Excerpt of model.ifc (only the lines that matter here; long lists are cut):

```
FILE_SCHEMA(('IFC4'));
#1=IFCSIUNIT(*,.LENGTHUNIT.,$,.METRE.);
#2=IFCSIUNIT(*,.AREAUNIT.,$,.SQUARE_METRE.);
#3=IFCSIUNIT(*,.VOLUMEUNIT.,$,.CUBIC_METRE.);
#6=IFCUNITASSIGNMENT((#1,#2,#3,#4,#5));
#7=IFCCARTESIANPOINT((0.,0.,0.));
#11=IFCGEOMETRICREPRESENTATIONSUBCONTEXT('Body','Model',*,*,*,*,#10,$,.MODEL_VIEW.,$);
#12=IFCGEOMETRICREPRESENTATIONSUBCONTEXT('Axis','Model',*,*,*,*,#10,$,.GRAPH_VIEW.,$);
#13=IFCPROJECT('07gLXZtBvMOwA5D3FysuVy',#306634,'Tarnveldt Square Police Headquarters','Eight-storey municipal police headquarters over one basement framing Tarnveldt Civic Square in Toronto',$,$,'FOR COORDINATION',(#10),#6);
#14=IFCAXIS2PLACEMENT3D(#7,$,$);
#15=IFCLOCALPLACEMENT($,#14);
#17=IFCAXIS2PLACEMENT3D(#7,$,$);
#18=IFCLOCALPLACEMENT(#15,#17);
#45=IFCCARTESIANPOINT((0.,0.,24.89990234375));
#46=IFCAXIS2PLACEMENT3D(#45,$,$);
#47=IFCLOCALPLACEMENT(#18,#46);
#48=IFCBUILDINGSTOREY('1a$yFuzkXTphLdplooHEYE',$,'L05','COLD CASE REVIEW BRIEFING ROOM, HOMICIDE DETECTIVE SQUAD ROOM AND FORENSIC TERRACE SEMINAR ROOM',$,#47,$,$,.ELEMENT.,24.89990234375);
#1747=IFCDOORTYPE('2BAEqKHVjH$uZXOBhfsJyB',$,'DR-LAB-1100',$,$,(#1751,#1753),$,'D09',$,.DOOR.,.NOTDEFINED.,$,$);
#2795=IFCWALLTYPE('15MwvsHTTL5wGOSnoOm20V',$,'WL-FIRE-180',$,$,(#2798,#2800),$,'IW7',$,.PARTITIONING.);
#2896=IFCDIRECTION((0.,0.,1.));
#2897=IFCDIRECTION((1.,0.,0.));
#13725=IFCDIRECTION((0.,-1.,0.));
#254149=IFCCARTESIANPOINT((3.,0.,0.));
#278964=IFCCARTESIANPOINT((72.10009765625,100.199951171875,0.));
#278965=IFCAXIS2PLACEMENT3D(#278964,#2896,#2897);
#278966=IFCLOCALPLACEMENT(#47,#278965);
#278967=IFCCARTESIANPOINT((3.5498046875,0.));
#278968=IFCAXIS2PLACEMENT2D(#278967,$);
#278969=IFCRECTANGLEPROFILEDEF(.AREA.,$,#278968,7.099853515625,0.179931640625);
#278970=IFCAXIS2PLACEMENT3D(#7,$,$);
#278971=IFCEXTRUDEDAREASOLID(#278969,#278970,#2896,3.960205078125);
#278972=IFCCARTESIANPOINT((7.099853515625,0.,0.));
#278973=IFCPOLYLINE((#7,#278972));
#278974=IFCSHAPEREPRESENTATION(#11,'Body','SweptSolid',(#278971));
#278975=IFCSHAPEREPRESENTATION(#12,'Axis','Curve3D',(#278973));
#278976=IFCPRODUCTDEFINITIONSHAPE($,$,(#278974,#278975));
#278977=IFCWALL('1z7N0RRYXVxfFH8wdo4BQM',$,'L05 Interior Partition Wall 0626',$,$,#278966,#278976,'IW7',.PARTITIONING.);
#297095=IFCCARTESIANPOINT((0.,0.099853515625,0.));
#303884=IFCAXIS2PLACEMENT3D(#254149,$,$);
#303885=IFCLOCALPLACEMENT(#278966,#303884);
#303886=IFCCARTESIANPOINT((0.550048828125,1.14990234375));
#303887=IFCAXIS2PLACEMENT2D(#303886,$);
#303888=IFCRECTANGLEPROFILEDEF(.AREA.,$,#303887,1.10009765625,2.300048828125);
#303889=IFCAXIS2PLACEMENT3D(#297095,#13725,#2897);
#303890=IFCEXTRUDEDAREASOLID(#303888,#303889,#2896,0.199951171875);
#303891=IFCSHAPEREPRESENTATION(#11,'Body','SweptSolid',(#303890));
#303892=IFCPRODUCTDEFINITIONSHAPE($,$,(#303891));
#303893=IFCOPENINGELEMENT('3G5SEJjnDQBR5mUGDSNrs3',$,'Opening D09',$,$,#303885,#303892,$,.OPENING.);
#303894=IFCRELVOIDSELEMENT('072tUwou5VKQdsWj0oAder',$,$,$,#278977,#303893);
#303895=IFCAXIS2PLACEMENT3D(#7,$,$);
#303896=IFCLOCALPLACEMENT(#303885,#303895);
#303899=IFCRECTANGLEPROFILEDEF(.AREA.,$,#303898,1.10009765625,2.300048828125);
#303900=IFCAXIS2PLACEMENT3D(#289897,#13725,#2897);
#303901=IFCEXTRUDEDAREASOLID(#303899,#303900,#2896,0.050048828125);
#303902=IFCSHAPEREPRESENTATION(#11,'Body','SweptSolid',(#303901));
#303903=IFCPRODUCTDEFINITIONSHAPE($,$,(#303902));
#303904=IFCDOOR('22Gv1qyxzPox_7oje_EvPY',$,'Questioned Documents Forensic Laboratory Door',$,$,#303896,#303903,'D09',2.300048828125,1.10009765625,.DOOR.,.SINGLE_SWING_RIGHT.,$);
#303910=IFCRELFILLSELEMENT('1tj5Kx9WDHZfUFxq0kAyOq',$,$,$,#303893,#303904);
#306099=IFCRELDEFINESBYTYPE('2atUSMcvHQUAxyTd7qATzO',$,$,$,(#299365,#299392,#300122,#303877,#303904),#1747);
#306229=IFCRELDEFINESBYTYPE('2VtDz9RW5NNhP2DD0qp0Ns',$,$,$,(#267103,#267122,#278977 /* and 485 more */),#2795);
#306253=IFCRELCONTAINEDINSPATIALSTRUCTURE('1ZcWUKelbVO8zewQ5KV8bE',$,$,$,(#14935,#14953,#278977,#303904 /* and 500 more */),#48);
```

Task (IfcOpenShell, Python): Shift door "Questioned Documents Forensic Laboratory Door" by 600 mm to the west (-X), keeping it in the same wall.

```python
import ifcopenshell
import ifcopenshell.api.geometry
import ifcopenshell.util.placement

model = ifcopenshell.open("model.ifc")

door = model.by_guid("22Gv1qyxzPox_7oje_EvPY")
opening = door.FillsVoids[0].RelatingOpeningElement
wall = opening.VoidsElements[0].RelatingBuildingElement

wall_matrix = ifcopenshell.util.placement.get_local_placement(wall.ObjectPlacement)
shift = wall_matrix[:3, 0] * -0.6
before = ifcopenshell.util.placement.get_local_placement(door.ObjectPlacement)[:3, 3].copy()

# The door is placed relative to its opening, so it follows when the opening moves.
matrix = ifcopenshell.util.placement.get_local_placement(opening.ObjectPlacement)
matrix[:3, 3] += shift
ifcopenshell.api.geometry.edit_object_placement(
    model, product=opening, matrix=matrix, is_si=False, should_transform_children=True
)

after = ifcopenshell.util.placement.get_local_placement(door.ObjectPlacement)[:3, 3]
print("door moved by", (after - before).round(3) + 0.0)

model.write("model_rev.ifc")
```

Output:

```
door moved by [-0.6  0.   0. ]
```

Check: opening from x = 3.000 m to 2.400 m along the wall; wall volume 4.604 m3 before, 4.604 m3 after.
